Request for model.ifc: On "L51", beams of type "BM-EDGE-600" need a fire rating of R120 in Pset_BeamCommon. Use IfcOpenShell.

First a look at what the model holds.

```python
import ifcopenshell
import ifcopenshell.util.element

model = ifcopenshell.open("model.ifc")
print(model.schema)
storey = next(s for s in model.by_type("IfcBuildingStorey") if s.Name == "L51")
beams = [e for e in ifcopenshell.util.element.get_decomposition(storey) if e.is_a("IfcBeam")]
seen = {}
for e in beams:
    element_type = ifcopenshell.util.element.get_type(e)
    key = (element_type.Name if element_type != e and element_type else None, ifcopenshell.util.element.get_pset(e, "Pset_BeamCommon", "FireRating"))
    seen[key] = seen.get(key, 0) + 1
for (name, value), count in sorted(seen.items(), key=str):
    print(count, "x", name, "|", value)
```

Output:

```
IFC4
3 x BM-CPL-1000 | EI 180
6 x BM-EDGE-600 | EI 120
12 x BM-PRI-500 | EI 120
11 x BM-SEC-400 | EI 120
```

```python
import ifcopenshell
import ifcopenshell.api.pset
import ifcopenshell.util.element

model = ifcopenshell.open("model.ifc")

storey = next(s for s in model.by_type("IfcBuildingStorey") if s.Name == "L51")
beams = [e for e in ifcopenshell.util.element.get_decomposition(storey) if e.is_a("IfcBeam")]

count = 0
for e in beams:
    element_type = ifcopenshell.util.element.get_type(e)
    if element_type in (None, e) or element_type.Name != "BM-EDGE-600":
        continue
    found = ifcopenshell.util.element.get_pset(e, "Pset_BeamCommon", should_inherit=False)
    if found:
        pset = model.by_id(found["id"])
        if len(ifcopenshell.util.element.get_elements_by_pset(pset)) > 1:
            pset = ifcopenshell.api.pset.unshare_pset(model, products=[e], pset=pset)[0]
    else:
        pset = ifcopenshell.api.pset.add_pset(model, product=e, name="Pset_BeamCommon")
    ifcopenshell.api.pset.edit_pset(model, pset=pset, properties={"FireRating": "R120"})
    count += 1

print(count, "beams updated")

model.write("model_v2.ifc")
```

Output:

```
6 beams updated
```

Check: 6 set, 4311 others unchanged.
